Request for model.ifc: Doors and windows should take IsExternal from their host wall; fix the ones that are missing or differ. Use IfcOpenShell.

First a look at what the model holds.

```python
import ifcopenshell
import ifcopenshell.util.element

model = ifcopenshell.open("model.ifc")
print(model.schema)
seen = {}
for e in model.by_type("IfcDoor") + model.by_type("IfcWindow"):
    if not e.FillsVoids:
        continue
    host = e.FillsVoids[0].RelatingOpeningElement.VoidsElements[0].RelatingBuildingElement
    own = ifcopenshell.util.element.get_pset(e, f"Pset_{e.is_a()[3:].removesuffix('StandardCase')}Common", "IsExternal")
    wall = ifcopenshell.util.element.get_pset(host, "Pset_WallCommon", "IsExternal")
    seen[e.is_a(), own, wall] = seen.get((e.is_a(), own, wall), 0) + 1
for (cls, own, wall), count in sorted(seen.items(), key=str):
    print(count, cls, "IsExternal:", own, "| host wall:", wall)
```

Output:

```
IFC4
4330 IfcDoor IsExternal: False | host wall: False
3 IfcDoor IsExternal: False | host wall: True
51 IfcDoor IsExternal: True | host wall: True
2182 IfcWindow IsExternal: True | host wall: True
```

```python
import ifcopenshell
import ifcopenshell.api.pset
import ifcopenshell.util.element

model = ifcopenshell.open("model.ifc")

count = 0
for ifc_class, pset_name in (("IfcDoor", "Pset_DoorCommon"), ("IfcWindow", "Pset_WindowCommon")):
    for e in model.by_type(ifc_class):
        if not e.FillsVoids:
            continue
        host = e.FillsVoids[0].RelatingOpeningElement.VoidsElements[0].RelatingBuildingElement
        external = ifcopenshell.util.element.get_pset(host, "Pset_WallCommon", "IsExternal")
        if external is None or ifcopenshell.util.element.get_pset(e, pset_name, "IsExternal") == external:
            continue
        pset = ifcopenshell.api.pset.add_pset(model, product=e, name=pset_name)
        ifcopenshell.api.pset.edit_pset(model, pset=pset, properties={"IsExternal": external})
        count += 1

print(count, "updated")

model.write("model_rev.ifc")
```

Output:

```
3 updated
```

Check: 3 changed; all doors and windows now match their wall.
